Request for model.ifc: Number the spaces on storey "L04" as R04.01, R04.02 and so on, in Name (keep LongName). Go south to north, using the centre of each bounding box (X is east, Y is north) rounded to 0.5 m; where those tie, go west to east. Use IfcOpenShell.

First a look at what the model holds.

```python
import ifcopenshell
import ifcopenshell.util.element
import ifcopenshell.util.placement

model = ifcopenshell.open("model.ifc")
print(model.schema)
storey = next(s for s in model.by_type("IfcBuildingStorey") if s.Name == "L04")
spaces = [e for e in ifcopenshell.util.element.get_decomposition(storey) if e.is_a("IfcSpace")]
for e in sorted(spaces, key=lambda e: e.id()):
    origin = ifcopenshell.util.placement.get_local_placement(e.ObjectPlacement)[:3, 3]
    print(e.id(), e.Name, e.LongName, origin.round(2) + 0.0, sep=" | ")
```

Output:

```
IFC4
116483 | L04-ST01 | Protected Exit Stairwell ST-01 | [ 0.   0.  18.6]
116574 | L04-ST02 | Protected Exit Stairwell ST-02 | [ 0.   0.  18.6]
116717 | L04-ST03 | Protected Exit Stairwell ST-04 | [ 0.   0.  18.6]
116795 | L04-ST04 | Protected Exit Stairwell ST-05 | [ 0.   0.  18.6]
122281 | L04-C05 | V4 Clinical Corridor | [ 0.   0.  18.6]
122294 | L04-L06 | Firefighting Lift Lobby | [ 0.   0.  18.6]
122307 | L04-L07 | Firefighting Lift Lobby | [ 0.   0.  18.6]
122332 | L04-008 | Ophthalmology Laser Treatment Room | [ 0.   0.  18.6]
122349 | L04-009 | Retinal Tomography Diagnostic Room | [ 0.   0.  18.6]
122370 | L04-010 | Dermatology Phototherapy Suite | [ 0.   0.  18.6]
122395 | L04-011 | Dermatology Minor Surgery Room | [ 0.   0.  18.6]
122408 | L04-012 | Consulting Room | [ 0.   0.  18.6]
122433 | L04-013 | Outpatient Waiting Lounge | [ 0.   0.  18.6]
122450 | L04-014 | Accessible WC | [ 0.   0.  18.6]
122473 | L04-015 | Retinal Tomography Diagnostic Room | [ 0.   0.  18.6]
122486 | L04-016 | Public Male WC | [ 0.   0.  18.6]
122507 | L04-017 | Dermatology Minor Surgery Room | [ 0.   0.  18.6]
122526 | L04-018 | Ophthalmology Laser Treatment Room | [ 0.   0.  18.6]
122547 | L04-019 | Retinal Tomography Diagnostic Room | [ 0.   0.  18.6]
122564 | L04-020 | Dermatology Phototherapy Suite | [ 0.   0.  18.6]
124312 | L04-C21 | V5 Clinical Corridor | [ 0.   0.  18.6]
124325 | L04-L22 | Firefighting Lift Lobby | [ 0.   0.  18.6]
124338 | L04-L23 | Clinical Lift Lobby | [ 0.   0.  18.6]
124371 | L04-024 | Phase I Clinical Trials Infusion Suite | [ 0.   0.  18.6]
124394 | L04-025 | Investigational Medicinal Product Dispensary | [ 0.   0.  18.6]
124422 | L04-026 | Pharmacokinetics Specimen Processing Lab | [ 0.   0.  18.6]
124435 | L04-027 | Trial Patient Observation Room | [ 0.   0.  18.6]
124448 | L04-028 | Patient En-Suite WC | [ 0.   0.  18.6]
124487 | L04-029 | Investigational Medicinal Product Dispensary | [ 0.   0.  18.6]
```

```python
import ifcopenshell
import ifcopenshell.geom
import ifcopenshell.util.element
import ifcopenshell.util.shape

model = ifcopenshell.open("model.ifc")
settings = ifcopenshell.geom.settings()
settings.set("use-world-coords", True)


def centre(element):
    shape = ifcopenshell.geom.create_shape(settings, element)
    return ifcopenshell.util.shape.get_bbox_centroid(shape.geometry)


storey = next(s for s in model.by_type("IfcBuildingStorey") if s.Name == "L04")
spaces = [e for e in ifcopenshell.util.element.get_decomposition(storey) if e.is_a("IfcSpace")]

# Insertion points can sit at a corner or the storey origin, so sort by the geometry (in metres).
centres = {e: centre(e) for e in spaces}
spaces.sort(key=lambda e: (round(centres[e][1] / 0.5), centres[e][0]))

for i, e in enumerate(spaces, start=1):
    number = f"R04.{i:02d}"
    e.Name = number
    print(e.id(), number)

model.write("model_updated.ifc")
```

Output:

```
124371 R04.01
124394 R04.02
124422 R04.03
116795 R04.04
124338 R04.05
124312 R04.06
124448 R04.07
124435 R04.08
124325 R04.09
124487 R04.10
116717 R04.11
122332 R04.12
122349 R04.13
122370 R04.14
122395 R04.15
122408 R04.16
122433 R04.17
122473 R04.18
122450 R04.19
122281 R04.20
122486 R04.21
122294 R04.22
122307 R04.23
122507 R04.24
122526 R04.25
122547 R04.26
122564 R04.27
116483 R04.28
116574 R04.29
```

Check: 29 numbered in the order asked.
